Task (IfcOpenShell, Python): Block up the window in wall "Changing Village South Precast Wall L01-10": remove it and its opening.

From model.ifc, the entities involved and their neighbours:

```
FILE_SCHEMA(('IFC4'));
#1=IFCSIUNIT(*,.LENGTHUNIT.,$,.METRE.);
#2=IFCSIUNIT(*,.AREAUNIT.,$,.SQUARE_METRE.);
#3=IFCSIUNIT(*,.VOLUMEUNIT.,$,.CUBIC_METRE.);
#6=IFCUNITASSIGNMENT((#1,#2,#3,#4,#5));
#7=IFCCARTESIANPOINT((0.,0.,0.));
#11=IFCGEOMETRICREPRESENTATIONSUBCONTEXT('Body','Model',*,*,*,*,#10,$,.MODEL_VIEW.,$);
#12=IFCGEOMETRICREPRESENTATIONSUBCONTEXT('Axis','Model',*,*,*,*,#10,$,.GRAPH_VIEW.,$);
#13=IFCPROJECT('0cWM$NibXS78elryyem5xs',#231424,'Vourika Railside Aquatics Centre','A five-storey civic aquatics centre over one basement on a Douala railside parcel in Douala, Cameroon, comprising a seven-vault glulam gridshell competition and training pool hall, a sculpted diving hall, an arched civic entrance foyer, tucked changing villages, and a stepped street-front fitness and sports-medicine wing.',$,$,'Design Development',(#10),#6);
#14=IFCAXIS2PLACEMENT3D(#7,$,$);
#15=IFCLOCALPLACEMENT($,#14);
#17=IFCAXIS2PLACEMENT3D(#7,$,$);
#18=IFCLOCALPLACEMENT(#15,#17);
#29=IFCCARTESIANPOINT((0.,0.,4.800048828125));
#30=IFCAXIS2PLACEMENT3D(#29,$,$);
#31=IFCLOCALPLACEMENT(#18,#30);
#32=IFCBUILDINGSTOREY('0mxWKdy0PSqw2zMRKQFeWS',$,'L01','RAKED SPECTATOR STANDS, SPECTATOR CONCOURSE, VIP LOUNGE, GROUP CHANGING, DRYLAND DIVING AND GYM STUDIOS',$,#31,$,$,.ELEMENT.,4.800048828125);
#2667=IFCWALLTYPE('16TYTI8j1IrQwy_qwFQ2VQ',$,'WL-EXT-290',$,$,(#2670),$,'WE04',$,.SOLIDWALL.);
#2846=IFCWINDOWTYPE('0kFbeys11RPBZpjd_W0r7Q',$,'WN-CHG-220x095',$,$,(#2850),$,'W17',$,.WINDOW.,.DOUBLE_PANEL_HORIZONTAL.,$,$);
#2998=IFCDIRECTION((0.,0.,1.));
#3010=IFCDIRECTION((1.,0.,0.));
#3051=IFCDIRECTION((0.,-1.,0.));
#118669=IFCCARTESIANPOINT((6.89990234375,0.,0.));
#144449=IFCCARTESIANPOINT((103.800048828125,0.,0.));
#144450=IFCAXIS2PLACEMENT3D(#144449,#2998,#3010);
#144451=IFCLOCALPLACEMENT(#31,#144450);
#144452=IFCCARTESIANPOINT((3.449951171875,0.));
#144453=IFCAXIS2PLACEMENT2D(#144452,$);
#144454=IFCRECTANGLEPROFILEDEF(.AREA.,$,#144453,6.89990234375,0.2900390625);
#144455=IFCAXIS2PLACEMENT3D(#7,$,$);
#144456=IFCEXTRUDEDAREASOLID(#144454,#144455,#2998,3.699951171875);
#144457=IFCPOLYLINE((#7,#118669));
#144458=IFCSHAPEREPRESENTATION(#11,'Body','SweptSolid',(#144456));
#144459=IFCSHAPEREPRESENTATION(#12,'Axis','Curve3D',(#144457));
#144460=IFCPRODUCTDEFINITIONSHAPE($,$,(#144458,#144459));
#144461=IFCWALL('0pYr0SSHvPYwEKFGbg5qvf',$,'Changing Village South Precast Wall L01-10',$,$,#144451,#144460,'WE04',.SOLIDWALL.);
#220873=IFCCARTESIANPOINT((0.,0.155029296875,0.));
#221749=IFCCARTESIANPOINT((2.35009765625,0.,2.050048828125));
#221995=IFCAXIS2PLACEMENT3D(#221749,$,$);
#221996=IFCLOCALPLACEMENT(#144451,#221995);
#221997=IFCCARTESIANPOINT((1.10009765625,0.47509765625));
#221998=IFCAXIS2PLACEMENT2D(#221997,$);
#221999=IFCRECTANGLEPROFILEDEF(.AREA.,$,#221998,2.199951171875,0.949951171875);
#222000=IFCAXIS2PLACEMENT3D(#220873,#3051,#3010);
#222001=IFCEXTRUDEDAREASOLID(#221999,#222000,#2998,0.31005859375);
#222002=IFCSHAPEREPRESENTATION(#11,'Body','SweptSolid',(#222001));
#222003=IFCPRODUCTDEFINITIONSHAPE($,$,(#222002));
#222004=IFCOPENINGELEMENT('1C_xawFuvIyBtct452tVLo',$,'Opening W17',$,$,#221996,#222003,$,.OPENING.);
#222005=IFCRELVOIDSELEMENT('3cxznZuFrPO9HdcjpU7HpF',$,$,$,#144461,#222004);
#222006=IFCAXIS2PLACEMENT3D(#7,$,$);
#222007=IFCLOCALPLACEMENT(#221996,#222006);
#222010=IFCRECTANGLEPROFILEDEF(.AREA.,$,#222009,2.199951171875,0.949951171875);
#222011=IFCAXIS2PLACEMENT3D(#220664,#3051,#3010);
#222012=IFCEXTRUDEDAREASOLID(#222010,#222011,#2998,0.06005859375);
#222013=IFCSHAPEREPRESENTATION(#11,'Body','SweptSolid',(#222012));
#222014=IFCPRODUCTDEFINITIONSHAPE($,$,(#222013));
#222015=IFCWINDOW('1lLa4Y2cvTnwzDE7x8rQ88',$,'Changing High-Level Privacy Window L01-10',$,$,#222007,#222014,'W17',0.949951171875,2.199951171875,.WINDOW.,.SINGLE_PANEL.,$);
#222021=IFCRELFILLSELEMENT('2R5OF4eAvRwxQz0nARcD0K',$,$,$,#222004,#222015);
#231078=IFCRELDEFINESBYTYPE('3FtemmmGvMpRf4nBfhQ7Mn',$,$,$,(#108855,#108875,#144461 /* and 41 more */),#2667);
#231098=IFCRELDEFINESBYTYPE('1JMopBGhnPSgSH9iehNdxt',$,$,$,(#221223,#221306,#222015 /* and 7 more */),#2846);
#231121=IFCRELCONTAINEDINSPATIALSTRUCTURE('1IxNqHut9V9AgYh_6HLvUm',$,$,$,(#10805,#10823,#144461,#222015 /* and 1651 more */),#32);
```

```python
import ifcopenshell
import ifcopenshell.api.feature
import ifcopenshell.api.root
import ifcopenshell.geom
import ifcopenshell.util.shape

model = ifcopenshell.open("model.ifc")
settings = ifcopenshell.geom.settings()


def volume(element):
    """Net volume in cubic metres, openings subtracted."""
    shape = ifcopenshell.geom.create_shape(settings, element)
    return ifcopenshell.util.shape.get_volume(shape.geometry)


window = model.by_guid("1lLa4Y2cvTnwzDE7x8rQ88")
opening = window.FillsVoids[0].RelatingOpeningElement
wall = opening.VoidsElements[0].RelatingBuildingElement
before = volume(wall)

ifcopenshell.api.root.remove_product(model, product=window)
ifcopenshell.api.feature.remove_feature(model, feature=opening)

after = volume(wall)

print(f"wall volume {before:.3f} -> {after:.3f} m3")

model.write("model_updated.ifc")
```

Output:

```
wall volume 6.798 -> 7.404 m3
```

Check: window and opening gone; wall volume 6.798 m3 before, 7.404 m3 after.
